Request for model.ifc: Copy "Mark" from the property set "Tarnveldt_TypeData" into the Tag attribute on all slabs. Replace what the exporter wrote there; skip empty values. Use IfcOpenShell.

First a look at what the model holds.

```python
import ifcopenshell
import ifcopenshell.util.element

model = ifcopenshell.open("model.ifc")
print(model.schema)
slabs = model.by_type("IfcSlab")
print(len(slabs), "slabs")
for e in slabs[:8]:
    source = ifcopenshell.util.element.get_pset(e, "Tarnveldt_TypeData", "Mark")
    target = e.Tag
    print(e.id(), repr(source), repr(target), sep=" | ")
```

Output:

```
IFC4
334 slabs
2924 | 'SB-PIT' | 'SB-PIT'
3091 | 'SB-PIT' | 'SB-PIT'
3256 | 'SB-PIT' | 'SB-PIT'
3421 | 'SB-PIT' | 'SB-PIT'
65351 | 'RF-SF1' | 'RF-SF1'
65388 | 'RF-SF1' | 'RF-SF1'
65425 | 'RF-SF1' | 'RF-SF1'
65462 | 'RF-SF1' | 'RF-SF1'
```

```python
import ifcopenshell
import ifcopenshell.util.element

model = ifcopenshell.open("model.ifc")

count = 0
for e in model.by_type("IfcSlab"):
    value = ifcopenshell.util.element.get_pset(e, "Tarnveldt_TypeData", "Mark")
    current = e.Tag
    if not value or not value.strip() or current == value:
        continue
    e.Tag = value
    count += 1

print(count, "slabs updated")

model.write("model_edited.ifc")
```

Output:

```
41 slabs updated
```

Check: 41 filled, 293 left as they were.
